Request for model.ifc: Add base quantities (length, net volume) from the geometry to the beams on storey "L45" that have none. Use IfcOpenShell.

First a look at what the model holds.

```python
import ifcopenshell
import ifcopenshell.util.element
import ifcopenshell.util.unit

model = ifcopenshell.open("model.ifc")
print(model.schema)
for unit_type in ("LENGTHUNIT", "AREAUNIT", "VOLUMEUNIT"):
    print(unit_type, ifcopenshell.util.unit.calculate_unit_scale(model, unit_type))
storey = next(s for s in model.by_type("IfcBuildingStorey") if s.Name == "L45")
beams = [e for e in ifcopenshell.util.element.get_decomposition(storey) if e.is_a("IfcBeam")]
for e in sorted(beams, key=lambda e: e.id()):
    print(e.id(), e.is_a(), e.Name, list(ifcopenshell.util.element.get_psets(e, qtos_only=True)), sep=" | ")
```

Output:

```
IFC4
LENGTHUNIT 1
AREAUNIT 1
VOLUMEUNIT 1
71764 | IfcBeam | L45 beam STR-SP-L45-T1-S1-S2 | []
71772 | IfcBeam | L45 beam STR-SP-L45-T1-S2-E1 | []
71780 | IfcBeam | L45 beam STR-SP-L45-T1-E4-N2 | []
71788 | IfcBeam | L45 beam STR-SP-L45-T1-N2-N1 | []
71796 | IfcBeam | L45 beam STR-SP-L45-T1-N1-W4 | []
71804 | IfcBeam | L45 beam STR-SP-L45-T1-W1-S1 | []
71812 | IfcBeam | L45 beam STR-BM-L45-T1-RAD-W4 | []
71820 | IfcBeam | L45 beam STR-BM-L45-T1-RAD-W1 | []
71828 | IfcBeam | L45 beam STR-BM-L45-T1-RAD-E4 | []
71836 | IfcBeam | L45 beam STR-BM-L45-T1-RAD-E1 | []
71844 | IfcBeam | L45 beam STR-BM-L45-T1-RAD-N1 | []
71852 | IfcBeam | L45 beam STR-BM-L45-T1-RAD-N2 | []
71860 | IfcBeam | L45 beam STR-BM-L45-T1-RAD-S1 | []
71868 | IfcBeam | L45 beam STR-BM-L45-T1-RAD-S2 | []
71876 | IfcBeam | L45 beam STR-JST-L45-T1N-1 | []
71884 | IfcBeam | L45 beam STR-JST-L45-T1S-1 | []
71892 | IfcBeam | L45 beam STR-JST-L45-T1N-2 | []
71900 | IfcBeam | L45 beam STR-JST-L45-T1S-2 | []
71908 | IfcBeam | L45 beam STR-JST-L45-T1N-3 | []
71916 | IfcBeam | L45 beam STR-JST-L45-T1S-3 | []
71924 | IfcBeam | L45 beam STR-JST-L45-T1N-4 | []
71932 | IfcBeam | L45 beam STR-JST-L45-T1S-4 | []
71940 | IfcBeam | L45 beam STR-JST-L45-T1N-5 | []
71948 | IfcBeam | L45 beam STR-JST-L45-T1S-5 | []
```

```python
import ifcopenshell
import ifcopenshell.api.pset
import ifcopenshell.geom
import ifcopenshell.util.element
import ifcopenshell.util.shape
import ifcopenshell.util.unit

model = ifcopenshell.open("model.ifc")
unit_scale = ifcopenshell.util.unit.calculate_unit_scale(model)
volume_scale = ifcopenshell.util.unit.calculate_unit_scale(model, "VOLUMEUNIT")
settings = ifcopenshell.geom.settings()

storey = next(s for s in model.by_type("IfcBuildingStorey") if s.Name == "L45")
beams = [e for e in ifcopenshell.util.element.get_decomposition(storey) if e.is_a("IfcBeam")]

for e in sorted(beams, key=lambda e: e.id()):
    if ifcopenshell.util.element.get_psets(e, qtos_only=True, should_inherit=False):
        continue
    # Geometry comes back in metres, in the element's own axes.
    shape = ifcopenshell.geom.create_shape(settings, e)
    values = {
        "Length": ifcopenshell.util.shape.get_max_xyz(shape.geometry) / unit_scale,
        "NetVolume": ifcopenshell.util.shape.get_volume(shape.geometry) / volume_scale,
    }
    qto = ifcopenshell.api.pset.add_qto(model, product=e, name="Qto_BeamBaseQuantities")
    ifcopenshell.api.pset.edit_qto(model, qto=qto, properties=values)
    print(e.id(), {k: round(v, 3) for k, v in values.items()})

model.write("model_edited.ifc")
```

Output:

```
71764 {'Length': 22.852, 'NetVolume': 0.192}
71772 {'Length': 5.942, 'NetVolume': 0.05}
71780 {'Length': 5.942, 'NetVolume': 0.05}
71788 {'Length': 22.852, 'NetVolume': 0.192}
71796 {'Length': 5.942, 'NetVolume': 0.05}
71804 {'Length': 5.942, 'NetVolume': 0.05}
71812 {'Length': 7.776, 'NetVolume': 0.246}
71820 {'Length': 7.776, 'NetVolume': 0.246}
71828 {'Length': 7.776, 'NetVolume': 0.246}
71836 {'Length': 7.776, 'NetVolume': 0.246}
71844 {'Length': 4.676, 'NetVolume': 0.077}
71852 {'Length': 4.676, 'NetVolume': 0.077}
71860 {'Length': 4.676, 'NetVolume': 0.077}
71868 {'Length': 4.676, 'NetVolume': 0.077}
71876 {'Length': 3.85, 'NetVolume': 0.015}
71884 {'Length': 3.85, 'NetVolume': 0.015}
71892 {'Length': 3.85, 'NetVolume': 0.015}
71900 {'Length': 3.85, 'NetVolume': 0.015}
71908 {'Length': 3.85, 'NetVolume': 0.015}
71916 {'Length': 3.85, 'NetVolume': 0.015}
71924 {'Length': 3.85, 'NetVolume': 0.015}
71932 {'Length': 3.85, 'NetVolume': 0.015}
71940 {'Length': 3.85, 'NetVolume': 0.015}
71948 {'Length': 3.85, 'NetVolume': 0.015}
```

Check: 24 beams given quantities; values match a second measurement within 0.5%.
